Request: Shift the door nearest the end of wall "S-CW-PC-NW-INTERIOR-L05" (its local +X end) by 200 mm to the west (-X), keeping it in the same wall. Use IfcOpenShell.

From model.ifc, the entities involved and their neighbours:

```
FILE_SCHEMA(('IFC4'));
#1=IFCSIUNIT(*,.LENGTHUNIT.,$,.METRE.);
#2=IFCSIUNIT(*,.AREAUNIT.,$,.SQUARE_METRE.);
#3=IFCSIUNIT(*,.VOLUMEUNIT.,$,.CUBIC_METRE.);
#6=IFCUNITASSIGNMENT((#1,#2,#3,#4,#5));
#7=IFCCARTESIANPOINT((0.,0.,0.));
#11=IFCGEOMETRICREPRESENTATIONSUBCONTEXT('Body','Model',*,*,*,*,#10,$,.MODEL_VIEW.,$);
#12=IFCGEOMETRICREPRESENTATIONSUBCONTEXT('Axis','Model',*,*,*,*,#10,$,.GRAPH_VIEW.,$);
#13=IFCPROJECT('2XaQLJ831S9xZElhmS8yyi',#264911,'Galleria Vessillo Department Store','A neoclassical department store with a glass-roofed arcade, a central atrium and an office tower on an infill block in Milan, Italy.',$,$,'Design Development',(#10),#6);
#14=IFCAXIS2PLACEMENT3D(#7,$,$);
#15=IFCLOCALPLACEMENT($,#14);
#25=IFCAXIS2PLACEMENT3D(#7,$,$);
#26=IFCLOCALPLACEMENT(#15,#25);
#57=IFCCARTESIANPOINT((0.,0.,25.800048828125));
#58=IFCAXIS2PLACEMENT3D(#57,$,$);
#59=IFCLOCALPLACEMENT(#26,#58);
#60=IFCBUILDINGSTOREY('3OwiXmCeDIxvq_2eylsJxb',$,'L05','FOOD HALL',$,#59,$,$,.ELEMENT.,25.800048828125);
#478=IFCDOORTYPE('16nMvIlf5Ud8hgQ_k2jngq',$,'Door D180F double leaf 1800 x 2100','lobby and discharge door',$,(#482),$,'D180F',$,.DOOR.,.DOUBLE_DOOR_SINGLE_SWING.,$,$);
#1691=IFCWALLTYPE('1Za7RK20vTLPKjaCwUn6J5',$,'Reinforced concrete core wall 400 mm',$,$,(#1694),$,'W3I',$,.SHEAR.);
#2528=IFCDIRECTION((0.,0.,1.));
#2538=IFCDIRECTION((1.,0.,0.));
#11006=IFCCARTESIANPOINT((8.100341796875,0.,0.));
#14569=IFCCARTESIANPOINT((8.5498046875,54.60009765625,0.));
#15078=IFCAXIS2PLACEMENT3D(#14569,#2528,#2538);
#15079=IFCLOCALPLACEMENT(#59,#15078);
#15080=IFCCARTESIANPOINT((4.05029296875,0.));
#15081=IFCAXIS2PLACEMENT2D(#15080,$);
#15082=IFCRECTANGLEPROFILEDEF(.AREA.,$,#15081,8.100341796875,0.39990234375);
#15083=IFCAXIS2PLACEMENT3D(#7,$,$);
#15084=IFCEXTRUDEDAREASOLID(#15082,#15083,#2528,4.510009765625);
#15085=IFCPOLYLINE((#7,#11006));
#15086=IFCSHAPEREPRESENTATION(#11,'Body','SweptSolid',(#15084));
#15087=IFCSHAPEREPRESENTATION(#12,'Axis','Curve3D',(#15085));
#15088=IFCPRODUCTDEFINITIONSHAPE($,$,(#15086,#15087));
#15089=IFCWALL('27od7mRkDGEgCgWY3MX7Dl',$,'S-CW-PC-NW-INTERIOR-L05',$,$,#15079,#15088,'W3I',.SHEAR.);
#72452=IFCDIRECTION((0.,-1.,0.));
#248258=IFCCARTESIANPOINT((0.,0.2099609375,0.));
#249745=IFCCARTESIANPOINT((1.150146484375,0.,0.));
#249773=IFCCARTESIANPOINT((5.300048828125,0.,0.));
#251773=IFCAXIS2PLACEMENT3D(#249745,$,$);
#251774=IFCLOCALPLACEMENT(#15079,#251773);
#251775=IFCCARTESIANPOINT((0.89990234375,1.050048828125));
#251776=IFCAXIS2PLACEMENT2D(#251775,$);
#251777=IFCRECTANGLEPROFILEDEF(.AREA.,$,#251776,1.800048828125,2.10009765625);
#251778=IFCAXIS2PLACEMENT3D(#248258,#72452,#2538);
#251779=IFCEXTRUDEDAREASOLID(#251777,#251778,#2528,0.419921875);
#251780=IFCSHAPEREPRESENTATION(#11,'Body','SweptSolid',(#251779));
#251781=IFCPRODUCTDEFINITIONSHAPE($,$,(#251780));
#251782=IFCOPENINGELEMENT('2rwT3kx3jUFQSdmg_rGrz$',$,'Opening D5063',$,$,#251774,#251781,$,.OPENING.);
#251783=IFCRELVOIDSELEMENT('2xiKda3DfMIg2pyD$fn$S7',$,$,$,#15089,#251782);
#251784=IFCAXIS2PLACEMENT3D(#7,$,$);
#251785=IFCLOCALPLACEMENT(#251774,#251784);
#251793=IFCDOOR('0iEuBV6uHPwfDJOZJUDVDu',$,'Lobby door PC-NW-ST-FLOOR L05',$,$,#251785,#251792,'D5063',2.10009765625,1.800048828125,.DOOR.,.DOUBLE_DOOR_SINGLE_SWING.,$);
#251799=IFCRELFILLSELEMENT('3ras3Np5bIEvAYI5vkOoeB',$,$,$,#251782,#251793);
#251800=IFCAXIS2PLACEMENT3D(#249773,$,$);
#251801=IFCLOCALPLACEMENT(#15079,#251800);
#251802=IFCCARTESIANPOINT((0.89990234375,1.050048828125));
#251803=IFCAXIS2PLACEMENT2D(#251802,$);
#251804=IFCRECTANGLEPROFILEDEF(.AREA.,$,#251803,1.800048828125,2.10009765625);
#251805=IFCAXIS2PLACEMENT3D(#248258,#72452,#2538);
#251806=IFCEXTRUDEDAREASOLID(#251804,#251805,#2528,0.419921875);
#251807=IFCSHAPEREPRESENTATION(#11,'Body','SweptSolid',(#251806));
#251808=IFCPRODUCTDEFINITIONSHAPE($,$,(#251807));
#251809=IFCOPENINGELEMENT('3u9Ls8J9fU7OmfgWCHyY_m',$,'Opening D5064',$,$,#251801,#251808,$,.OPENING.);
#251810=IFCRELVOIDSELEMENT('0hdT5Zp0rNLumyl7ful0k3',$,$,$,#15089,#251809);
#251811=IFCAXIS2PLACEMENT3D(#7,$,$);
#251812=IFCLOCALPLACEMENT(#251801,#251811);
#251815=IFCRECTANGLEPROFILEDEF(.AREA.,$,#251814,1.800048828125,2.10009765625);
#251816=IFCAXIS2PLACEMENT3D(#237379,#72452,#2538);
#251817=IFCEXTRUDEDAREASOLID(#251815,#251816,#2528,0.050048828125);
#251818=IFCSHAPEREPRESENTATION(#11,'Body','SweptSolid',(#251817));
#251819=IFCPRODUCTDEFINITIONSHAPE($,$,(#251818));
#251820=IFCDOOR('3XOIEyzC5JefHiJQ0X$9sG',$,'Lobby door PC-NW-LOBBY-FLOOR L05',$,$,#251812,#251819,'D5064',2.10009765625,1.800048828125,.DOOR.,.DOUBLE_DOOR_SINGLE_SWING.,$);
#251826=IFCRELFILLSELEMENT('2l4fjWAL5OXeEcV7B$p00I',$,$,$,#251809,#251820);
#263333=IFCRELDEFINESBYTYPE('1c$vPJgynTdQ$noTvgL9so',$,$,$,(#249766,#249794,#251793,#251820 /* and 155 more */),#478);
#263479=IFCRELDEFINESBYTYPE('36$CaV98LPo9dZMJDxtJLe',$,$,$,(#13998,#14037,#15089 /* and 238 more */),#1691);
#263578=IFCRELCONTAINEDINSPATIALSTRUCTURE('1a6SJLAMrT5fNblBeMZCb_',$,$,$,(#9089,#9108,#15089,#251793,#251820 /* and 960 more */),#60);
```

```python
import ifcopenshell
import ifcopenshell.api.geometry
import ifcopenshell.util.placement
import ifcopenshell.util.unit

model = ifcopenshell.open("model.ifc")
unit_scale = ifcopenshell.util.unit.calculate_unit_scale(model)

door = model.by_guid("3XOIEyzC5JefHiJQ0X$9sG")
opening = door.FillsVoids[0].RelatingOpeningElement
wall = opening.VoidsElements[0].RelatingBuildingElement

wall_matrix = ifcopenshell.util.placement.get_local_placement(wall.ObjectPlacement)
shift = wall_matrix[:3, 0] * -0.2 / unit_scale
before = ifcopenshell.util.placement.get_local_placement(door.ObjectPlacement)[:3, 3].copy()

# The door is placed relative to its opening, so it follows when the opening moves.
matrix = ifcopenshell.util.placement.get_local_placement(opening.ObjectPlacement)
matrix[:3, 3] += shift
ifcopenshell.api.geometry.edit_object_placement(
    model, product=opening, matrix=matrix, is_si=False, should_transform_children=True
)

after = ifcopenshell.util.placement.get_local_placement(door.ObjectPlacement)[:3, 3]
print("door moved by", (after - before).round(3) + 0.0)

model.write("model-out.ifc")
```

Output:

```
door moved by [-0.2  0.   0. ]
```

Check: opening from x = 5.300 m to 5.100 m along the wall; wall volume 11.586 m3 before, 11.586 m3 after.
